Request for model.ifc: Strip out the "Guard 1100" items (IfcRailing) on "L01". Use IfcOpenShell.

First a look at what the model holds.

```python
import ifcopenshell
import ifcopenshell.util.element

model = ifcopenshell.open("model.ifc")
print(model.schema)
storey = next(s for s in model.by_type("IfcBuildingStorey") if s.Name == "L01")
railings = [e for e in ifcopenshell.util.element.get_decomposition(storey) if e.is_a("IfcRailing")]
seen = {}
for e in railings:
    element_type = ifcopenshell.util.element.get_type(e)
    name = element_type.Name if element_type not in (None, e) else None
    seen[name] = seen.get(name, 0) + 1
for name, count in sorted(seen.items(), key=str):
    print(count, "x", name)
```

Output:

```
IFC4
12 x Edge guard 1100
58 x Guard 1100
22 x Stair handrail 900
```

```python
import ifcopenshell
import ifcopenshell.api.root
import ifcopenshell.util.element

model = ifcopenshell.open("model.ifc")

storey = next(s for s in model.by_type("IfcBuildingStorey") if s.Name == "L01")
railings = [e for e in ifcopenshell.util.element.get_decomposition(storey) if e.is_a("IfcRailing")]
targets = [e for e in railings if (t := ifcopenshell.util.element.get_type(e)) not in (None, e) and t.Name == "Guard 1100"]

for e in targets:
    ifcopenshell.api.root.remove_product(model, product=e)
print(len(targets), "removed")

model.write("model_updated.ifc")
```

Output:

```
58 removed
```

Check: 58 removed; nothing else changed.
